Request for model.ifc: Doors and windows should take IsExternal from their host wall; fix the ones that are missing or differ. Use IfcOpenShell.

First a look at what the model holds.

```python
import ifcopenshell
import ifcopenshell.util.element

model = ifcopenshell.open("model.ifc")
print(model.schema)
seen = {}
for e in model.by_type("IfcDoor") + model.by_type("IfcWindow"):
    if not e.FillsVoids:
        continue
    host = e.FillsVoids[0].RelatingOpeningElement.VoidsElements[0].RelatingBuildingElement
    own = ifcopenshell.util.element.get_pset(e, f"Pset_{e.is_a()[3:].removesuffix('StandardCase')}Common", "IsExternal")
    wall = ifcopenshell.util.element.get_pset(host, "Pset_WallCommon", "IsExternal")
    seen[e.is_a(), own, wall] = seen.get((e.is_a(), own, wall), 0) + 1
for (cls, own, wall), count in sorted(seen.items(), key=str):
    print(count, cls, "IsExternal:", own, "| host wall:", wall)
```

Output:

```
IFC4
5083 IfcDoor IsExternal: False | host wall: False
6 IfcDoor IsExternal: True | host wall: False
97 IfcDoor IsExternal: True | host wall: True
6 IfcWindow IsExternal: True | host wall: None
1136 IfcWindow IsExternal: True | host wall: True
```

```python
import ifcopenshell
import ifcopenshell.api.pset
import ifcopenshell.util.element

model = ifcopenshell.open("model.ifc")

count = 0
for ifc_class, pset_name in (("IfcDoor", "Pset_DoorCommon"), ("IfcWindow", "Pset_WindowCommon")):
    for e in model.by_type(ifc_class):
        if not e.FillsVoids:
            continue
        host = e.FillsVoids[0].RelatingOpeningElement.VoidsElements[0].RelatingBuildingElement
        external = ifcopenshell.util.element.get_pset(host, "Pset_WallCommon", "IsExternal")
        if external is None or ifcopenshell.util.element.get_pset(e, pset_name, "IsExternal") == external:
            continue
        found = ifcopenshell.util.element.get_pset(e, pset_name, should_inherit=False)
        if found:
            pset = model.by_id(found["id"])
            if len(ifcopenshell.util.element.get_elements_by_pset(pset)) > 1:
                pset = ifcopenshell.api.pset.unshare_pset(model, products=[e], pset=pset)[0]
        else:
            pset = ifcopenshell.api.pset.add_pset(model, product=e, name=pset_name)
        ifcopenshell.api.pset.edit_pset(model, pset=pset, properties={"IsExternal": external})
        count += 1

print(count, "updated")

model.write("model_updated.ifc")
```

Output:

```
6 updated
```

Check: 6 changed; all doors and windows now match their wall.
